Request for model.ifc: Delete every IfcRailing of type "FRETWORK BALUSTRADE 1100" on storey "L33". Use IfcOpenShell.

First a look at what the model holds.

```python
import ifcopenshell
import ifcopenshell.util.element

model = ifcopenshell.open("model.ifc")
print(model.schema)
storey = next(s for s in model.by_type("IfcBuildingStorey") if s.Name == "L33")
railings = [e for e in ifcopenshell.util.element.get_decomposition(storey) if e.is_a("IfcRailing")]
seen = {}
for e in railings:
    element_type = ifcopenshell.util.element.get_type(e)
    name = element_type.Name if element_type not in (None, e) else None
    seen[name] = seen.get(name, 0) + 1
for name, count in sorted(seen.items(), key=str):
    print(count, "x", name)
```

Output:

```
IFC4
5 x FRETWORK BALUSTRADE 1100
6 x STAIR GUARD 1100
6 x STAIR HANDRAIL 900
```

```python
import ifcopenshell
import ifcopenshell.api.root
import ifcopenshell.util.element

model = ifcopenshell.open("model.ifc")

storey = next(s for s in model.by_type("IfcBuildingStorey") if s.Name == "L33")
railings = [e for e in ifcopenshell.util.element.get_decomposition(storey) if e.is_a("IfcRailing")]
targets = [e for e in railings if (t := ifcopenshell.util.element.get_type(e)) not in (None, e) and t.Name == "FRETWORK BALUSTRADE 1100"]

for e in targets:
    ifcopenshell.api.root.remove_product(model, product=e)
print(len(targets), "removed")

model.write("model_edited.ifc")
```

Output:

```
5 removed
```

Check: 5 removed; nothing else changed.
